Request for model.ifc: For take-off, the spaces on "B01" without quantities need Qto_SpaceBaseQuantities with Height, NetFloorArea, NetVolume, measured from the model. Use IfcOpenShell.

First a look at what the model holds.

```python
import ifcopenshell
import ifcopenshell.util.element
import ifcopenshell.util.unit

model = ifcopenshell.open("model.ifc")
print(model.schema)
for unit_type in ("LENGTHUNIT", "AREAUNIT", "VOLUMEUNIT"):
    print(unit_type, ifcopenshell.util.unit.calculate_unit_scale(model, unit_type))
storey = next(s for s in model.by_type("IfcBuildingStorey") if s.Name == "B01")
spaces = [e for e in ifcopenshell.util.element.get_decomposition(storey) if e.is_a("IfcSpace")]
for e in sorted(spaces, key=lambda e: e.id()):
    print(e.id(), e.is_a(), e.Name, list(ifcopenshell.util.element.get_psets(e, qtos_only=True)), sep=" | ")
```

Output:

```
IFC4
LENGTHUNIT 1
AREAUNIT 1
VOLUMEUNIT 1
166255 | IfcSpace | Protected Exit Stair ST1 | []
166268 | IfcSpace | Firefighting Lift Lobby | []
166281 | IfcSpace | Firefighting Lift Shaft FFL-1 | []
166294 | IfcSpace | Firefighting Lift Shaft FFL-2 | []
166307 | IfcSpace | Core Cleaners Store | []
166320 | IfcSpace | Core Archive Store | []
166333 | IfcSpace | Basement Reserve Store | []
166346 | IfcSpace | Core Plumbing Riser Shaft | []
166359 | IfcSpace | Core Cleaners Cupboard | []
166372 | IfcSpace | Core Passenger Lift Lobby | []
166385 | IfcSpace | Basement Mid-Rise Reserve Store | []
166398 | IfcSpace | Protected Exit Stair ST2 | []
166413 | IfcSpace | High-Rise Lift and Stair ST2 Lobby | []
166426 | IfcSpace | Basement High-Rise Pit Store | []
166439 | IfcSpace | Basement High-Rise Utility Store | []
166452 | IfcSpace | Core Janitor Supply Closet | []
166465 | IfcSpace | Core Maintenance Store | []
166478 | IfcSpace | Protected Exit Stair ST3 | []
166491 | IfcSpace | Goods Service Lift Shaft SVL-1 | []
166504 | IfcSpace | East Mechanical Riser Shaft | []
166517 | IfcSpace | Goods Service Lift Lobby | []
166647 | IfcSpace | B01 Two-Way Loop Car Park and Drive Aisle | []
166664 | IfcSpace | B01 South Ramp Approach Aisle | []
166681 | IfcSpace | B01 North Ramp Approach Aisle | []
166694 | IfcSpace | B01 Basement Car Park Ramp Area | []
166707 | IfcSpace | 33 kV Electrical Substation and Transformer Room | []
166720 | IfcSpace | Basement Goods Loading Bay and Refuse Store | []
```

```python
import ifcopenshell
import ifcopenshell.api.pset
import ifcopenshell.geom
import ifcopenshell.util.element
import ifcopenshell.util.shape
import ifcopenshell.util.unit

model = ifcopenshell.open("model.ifc")
unit_scale = ifcopenshell.util.unit.calculate_unit_scale(model)
area_scale = ifcopenshell.util.unit.calculate_unit_scale(model, "AREAUNIT")
volume_scale = ifcopenshell.util.unit.calculate_unit_scale(model, "VOLUMEUNIT")
settings = ifcopenshell.geom.settings()

storey = next(s for s in model.by_type("IfcBuildingStorey") if s.Name == "B01")
spaces = [e for e in ifcopenshell.util.element.get_decomposition(storey) if e.is_a("IfcSpace")]

for e in sorted(spaces, key=lambda e: e.id()):
    if ifcopenshell.util.element.get_psets(e, qtos_only=True, should_inherit=False):
        continue
    # Geometry comes back in metres, in the element's own axes.
    shape = ifcopenshell.geom.create_shape(settings, e)
    values = {
        "Height": ifcopenshell.util.shape.get_z(shape.geometry) / unit_scale,
        "NetFloorArea": ifcopenshell.util.shape.get_footprint_area(shape.geometry) / area_scale,
        "NetVolume": ifcopenshell.util.shape.get_volume(shape.geometry) / volume_scale,
    }
    qto = ifcopenshell.api.pset.add_qto(model, product=e, name="Qto_SpaceBaseQuantities")
    ifcopenshell.api.pset.edit_qto(model, qto=qto, properties=values)
    print(e.id(), {k: round(v, 3) for k, v in values.items()})

model.write("model_v2.ifc")
```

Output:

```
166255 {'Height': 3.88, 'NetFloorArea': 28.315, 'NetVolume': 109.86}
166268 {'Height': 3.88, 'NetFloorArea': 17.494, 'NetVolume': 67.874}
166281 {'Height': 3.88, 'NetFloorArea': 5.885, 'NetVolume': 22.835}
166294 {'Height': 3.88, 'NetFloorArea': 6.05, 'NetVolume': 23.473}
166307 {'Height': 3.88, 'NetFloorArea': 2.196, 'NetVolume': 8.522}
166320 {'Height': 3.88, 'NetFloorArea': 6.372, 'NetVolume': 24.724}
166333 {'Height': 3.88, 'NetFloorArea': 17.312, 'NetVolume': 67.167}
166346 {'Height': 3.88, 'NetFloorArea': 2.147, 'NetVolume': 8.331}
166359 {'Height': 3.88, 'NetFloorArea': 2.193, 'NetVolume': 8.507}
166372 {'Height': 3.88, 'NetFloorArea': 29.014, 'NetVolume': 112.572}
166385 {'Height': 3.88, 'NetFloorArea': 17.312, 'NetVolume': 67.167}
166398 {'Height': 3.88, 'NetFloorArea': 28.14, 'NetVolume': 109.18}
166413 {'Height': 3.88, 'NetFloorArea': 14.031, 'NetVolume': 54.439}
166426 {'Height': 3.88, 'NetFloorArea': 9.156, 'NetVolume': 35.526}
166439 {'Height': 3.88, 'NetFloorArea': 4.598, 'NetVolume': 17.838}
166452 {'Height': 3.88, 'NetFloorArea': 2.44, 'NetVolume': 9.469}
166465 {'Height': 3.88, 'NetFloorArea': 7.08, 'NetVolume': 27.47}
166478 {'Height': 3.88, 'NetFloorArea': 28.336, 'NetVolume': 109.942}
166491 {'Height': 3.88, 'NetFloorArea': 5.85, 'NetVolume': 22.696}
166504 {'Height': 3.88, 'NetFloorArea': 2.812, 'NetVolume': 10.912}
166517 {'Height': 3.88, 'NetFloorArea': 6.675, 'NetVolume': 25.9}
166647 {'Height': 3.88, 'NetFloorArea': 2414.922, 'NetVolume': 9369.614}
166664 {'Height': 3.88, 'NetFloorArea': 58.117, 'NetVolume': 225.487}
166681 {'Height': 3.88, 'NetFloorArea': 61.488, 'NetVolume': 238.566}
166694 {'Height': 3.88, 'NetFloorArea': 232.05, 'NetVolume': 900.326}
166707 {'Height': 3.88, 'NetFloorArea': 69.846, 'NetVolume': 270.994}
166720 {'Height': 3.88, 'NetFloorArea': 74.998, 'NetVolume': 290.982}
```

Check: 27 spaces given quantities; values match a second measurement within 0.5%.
